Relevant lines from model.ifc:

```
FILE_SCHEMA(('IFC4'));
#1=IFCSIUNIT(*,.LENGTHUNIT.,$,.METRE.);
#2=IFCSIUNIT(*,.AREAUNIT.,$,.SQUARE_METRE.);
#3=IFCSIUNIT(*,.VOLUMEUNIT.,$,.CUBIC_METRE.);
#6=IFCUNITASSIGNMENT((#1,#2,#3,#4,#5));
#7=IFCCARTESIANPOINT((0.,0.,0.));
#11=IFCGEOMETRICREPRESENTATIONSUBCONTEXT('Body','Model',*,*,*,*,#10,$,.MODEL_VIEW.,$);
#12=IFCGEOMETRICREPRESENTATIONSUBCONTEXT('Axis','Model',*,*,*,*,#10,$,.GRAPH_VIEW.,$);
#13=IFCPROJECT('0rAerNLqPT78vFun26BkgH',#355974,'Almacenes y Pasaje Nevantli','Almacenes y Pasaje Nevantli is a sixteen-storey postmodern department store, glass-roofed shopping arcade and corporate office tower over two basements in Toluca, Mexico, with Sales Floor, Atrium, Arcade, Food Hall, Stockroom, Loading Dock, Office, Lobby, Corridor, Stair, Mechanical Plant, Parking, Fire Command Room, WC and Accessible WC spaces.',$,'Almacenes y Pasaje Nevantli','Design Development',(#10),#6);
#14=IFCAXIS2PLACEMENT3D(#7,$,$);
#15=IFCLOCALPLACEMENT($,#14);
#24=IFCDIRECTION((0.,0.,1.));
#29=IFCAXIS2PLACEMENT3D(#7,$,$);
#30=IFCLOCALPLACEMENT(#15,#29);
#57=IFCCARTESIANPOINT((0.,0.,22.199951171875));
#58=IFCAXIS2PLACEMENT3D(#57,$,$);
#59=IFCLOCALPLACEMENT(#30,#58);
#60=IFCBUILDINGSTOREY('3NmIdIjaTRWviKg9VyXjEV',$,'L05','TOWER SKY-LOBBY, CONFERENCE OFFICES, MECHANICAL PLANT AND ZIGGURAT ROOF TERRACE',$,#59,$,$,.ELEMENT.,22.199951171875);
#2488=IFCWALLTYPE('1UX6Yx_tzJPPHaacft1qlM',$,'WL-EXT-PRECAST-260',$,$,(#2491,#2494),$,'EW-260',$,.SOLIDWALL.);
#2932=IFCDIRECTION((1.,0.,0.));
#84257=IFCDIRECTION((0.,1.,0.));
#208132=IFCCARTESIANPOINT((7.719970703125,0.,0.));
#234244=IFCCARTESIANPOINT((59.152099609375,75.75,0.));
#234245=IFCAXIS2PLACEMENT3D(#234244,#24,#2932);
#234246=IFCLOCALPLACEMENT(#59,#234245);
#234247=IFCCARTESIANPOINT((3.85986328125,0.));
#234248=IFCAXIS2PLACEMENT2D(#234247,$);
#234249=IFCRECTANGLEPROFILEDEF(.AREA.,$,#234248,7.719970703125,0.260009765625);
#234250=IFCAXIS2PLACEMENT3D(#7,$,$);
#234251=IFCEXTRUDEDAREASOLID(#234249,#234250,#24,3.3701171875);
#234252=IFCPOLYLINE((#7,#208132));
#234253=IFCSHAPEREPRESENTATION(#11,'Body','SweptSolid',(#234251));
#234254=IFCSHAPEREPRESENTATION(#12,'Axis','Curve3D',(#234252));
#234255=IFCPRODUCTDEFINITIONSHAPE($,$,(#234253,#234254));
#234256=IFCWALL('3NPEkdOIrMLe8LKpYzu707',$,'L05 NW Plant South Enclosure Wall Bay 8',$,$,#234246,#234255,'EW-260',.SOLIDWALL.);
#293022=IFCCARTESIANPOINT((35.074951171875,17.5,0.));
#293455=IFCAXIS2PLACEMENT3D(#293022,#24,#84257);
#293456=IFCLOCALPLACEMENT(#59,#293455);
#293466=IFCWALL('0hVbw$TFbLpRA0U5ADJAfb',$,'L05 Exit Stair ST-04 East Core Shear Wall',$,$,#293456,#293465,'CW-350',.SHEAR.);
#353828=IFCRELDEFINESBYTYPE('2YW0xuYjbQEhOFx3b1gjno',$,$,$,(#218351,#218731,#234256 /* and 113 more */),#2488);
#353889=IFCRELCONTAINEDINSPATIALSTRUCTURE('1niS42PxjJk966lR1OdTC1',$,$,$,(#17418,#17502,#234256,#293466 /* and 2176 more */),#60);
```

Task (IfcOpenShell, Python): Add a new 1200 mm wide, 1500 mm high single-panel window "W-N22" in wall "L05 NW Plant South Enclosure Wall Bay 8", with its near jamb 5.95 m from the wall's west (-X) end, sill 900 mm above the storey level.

```python
import numpy as np
import ifcopenshell
import ifcopenshell.api.feature
import ifcopenshell.api.geometry
import ifcopenshell.api.root
import ifcopenshell.api.spatial
import ifcopenshell.geom
import ifcopenshell.util.element
import ifcopenshell.util.placement
import ifcopenshell.util.representation
import ifcopenshell.util.shape
import ifcopenshell.util.unit

model = ifcopenshell.open("model.ifc")
unit_scale = ifcopenshell.util.unit.calculate_unit_scale(model)
settings = ifcopenshell.geom.settings()


def volume(element):
    """Net volume in cubic metres, openings subtracted."""
    shape = ifcopenshell.geom.create_shape(settings, element)
    return ifcopenshell.util.shape.get_volume(shape.geometry)


wall = model.by_id(234256)
storey = ifcopenshell.util.element.get_container(wall, ifc_class="IfcBuildingStorey")
context = ifcopenshell.util.representation.get_context(model, "Model", "Body", "MODEL_VIEW")
before = volume(wall)

width, height, from_end, sill = 1.2, 1.5, 5.95, 0.9  # metres

# The wall runs along its own X axis, and the end named is its -X end.
wall_shape = ifcopenshell.geom.create_shape(settings, wall)
x, y, z = ifcopenshell.util.shape.get_vertices(wall_shape.geometry).T
start = x.min() + from_end
face, thickness = float(y.min()), float(y.max() - y.min())
wall_matrix = ifcopenshell.util.placement.get_local_placement(wall.ObjectPlacement)
level = ifcopenshell.util.placement.get_local_placement(storey.ObjectPlacement)[2, 3]


def in_wall(x, y):
    """Placement at x, y metres in the wall's axes, at sill height."""
    matrix = wall_matrix.copy()
    matrix[:, 3] = wall_matrix @ np.array([x / unit_scale, y / unit_scale, 0.0, 1.0])
    matrix[2, 3] = level + sill / unit_scale
    return matrix


# Opening: a box that overshoots both wall faces by 50 mm.
opening = ifcopenshell.api.root.create_entity(model, ifc_class="IfcOpeningElement", predefined_type="OPENING")
box = ifcopenshell.api.geometry.add_wall_representation(
    model, context=context, length=width, height=height, thickness=thickness + 0.1
)
ifcopenshell.api.geometry.assign_representation(model, product=opening, representation=box)
ifcopenshell.api.geometry.edit_object_placement(model, product=opening, matrix=in_wall(start, face - 0.05), is_si=False)
ifcopenshell.api.feature.add_feature(model, feature=opening, element=wall)

window = ifcopenshell.api.root.create_entity(model, ifc_class="IfcWindow", name="W-N22", predefined_type="WINDOW")
window.OverallWidth, window.OverallHeight = width / unit_scale, height / unit_scale
window.PartitioningType = "SINGLE_PANEL"
body = ifcopenshell.api.geometry.add_window_representation(
    model,
    context=context,
    overall_width=window.OverallWidth,
    overall_height=window.OverallHeight,
    partition_type="SINGLE_PANEL",
)
ifcopenshell.api.geometry.assign_representation(model, product=window, representation=body)
ifcopenshell.api.spatial.assign_container(model, products=[window], relating_structure=storey)
ifcopenshell.api.feature.add_filling(model, opening=opening, element=window)

# Centre the window in the wall's thickness.
ifcopenshell.api.geometry.edit_object_placement(model, product=window, matrix=in_wall(start, face), is_si=False)
window_shape = ifcopenshell.geom.create_shape(settings, window)
depth = ifcopenshell.util.shape.get_vertices(window_shape.geometry)[:, 1]
offset = face + thickness / 2 - (depth.min() + depth.max()) / 2
ifcopenshell.api.geometry.edit_object_placement(model, product=window, matrix=in_wall(start, offset), is_si=False)

after = volume(wall)

print(f"wall volume {before:.3f} -> {after:.3f} m3")

model.write("model_rev.ifc")
```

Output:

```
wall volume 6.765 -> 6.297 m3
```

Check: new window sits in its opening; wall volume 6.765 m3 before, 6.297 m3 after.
